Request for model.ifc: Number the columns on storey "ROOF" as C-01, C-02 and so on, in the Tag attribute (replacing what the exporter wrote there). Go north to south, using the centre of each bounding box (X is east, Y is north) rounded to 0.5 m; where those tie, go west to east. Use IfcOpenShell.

First a look at what the model holds.

```python
import ifcopenshell
import ifcopenshell.util.element
import ifcopenshell.util.placement

model = ifcopenshell.open("model.ifc")
print(model.schema)
storey = next(s for s in model.by_type("IfcBuildingStorey") if s.Name == "ROOF")
columns = [e for e in ifcopenshell.util.element.get_decomposition(storey) if e.is_a("IfcColumn")]
for e in sorted(columns, key=lambda e: e.id()):
    origin = ifcopenshell.util.placement.get_local_placement(e.ObjectPlacement)[:3, 3]
    print(e.id(), e.Tag, e.Name, origin.round(2) + 0.0, sep=" | ")
```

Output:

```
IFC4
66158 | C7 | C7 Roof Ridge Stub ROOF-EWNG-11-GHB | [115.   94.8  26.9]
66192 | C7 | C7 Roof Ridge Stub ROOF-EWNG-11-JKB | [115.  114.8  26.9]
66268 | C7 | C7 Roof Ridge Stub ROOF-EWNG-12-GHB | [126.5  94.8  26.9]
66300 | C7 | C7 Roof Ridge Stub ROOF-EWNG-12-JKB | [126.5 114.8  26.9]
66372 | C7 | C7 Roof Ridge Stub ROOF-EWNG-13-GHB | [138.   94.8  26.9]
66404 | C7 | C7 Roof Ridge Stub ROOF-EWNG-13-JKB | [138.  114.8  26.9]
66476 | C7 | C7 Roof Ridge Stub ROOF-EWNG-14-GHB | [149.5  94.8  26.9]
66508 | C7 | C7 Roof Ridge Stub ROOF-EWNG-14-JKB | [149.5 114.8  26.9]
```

```python
import ifcopenshell
import ifcopenshell.geom
import ifcopenshell.util.element
import ifcopenshell.util.shape

model = ifcopenshell.open("model.ifc")
settings = ifcopenshell.geom.settings()
settings.set("use-world-coords", True)


def centre(element):
    shape = ifcopenshell.geom.create_shape(settings, element)
    return ifcopenshell.util.shape.get_bbox_centroid(shape.geometry)


storey = next(s for s in model.by_type("IfcBuildingStorey") if s.Name == "ROOF")
columns = [e for e in ifcopenshell.util.element.get_decomposition(storey) if e.is_a("IfcColumn")]

# Insertion points can sit at a corner or the storey origin, so sort by the geometry (in metres).
centres = {e: centre(e) for e in columns}
columns.sort(key=lambda e: (-round(centres[e][1] / 0.5), centres[e][0]))

for i, e in enumerate(columns, start=1):
    number = f"C-{i:02d}"
    e.Tag = number
    print(e.id(), number)

model.write("model-out.ifc")
```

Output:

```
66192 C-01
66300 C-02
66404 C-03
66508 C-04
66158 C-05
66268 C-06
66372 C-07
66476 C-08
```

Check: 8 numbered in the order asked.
